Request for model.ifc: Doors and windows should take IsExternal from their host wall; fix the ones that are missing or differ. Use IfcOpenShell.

First a look at what the model holds.

```python
import ifcopenshell
import ifcopenshell.util.element

model = ifcopenshell.open("model.ifc")
print(model.schema)
seen = {}
for e in model.by_type("IfcDoor") + model.by_type("IfcWindow"):
    if not e.FillsVoids:
        continue
    host = e.FillsVoids[0].RelatingOpeningElement.VoidsElements[0].RelatingBuildingElement
    own = ifcopenshell.util.element.get_pset(e, f"Pset_{e.is_a()[3:].removesuffix('StandardCase')}Common", "IsExternal")
    wall = ifcopenshell.util.element.get_pset(host, "Pset_WallCommon", "IsExternal")
    seen[e.is_a(), own, wall] = seen.get((e.is_a(), own, wall), 0) + 1
for (cls, own, wall), count in sorted(seen.items(), key=str):
    print(count, cls, "IsExternal:", own, "| host wall:", wall)
```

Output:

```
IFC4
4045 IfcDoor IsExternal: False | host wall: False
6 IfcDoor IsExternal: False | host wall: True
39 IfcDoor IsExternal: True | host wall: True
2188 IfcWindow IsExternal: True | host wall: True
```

```python
import ifcopenshell
import ifcopenshell.api.pset
import ifcopenshell.util.element

model = ifcopenshell.open("model.ifc")

count = 0
for ifc_class, pset_name in (("IfcDoor", "Pset_DoorCommon"), ("IfcWindow", "Pset_WindowCommon")):
    for e in model.by_type(ifc_class):
        if not e.FillsVoids:
            continue
        host = e.FillsVoids[0].RelatingOpeningElement.VoidsElements[0].RelatingBuildingElement
        external = ifcopenshell.util.element.get_pset(host, "Pset_WallCommon", "IsExternal")
        if external is None or ifcopenshell.util.element.get_pset(e, pset_name, "IsExternal") == external:
            continue
        pset = ifcopenshell.api.pset.add_pset(model, product=e, name=pset_name)
        ifcopenshell.api.pset.edit_pset(model, pset=pset, properties={"IsExternal": external})
        count += 1

print(count, "updated")

model.write("model_updated.ifc")
```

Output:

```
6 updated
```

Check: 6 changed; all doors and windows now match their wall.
